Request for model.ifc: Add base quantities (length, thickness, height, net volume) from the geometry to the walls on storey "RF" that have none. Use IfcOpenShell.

First a look at what the model holds.

```python
import ifcopenshell
import ifcopenshell.util.element
import ifcopenshell.util.unit

model = ifcopenshell.open("model.ifc")
print(model.schema)
for unit_type in ("LENGTHUNIT", "AREAUNIT", "VOLUMEUNIT"):
    print(unit_type, ifcopenshell.util.unit.calculate_unit_scale(model, unit_type))
storey = next(s for s in model.by_type("IfcBuildingStorey") if s.Name == "RF")
walls = [e for e in ifcopenshell.util.element.get_decomposition(storey) if e.is_a("IfcWall")]
for e in sorted(walls, key=lambda e: e.id()):
    print(e.id(), e.is_a(), e.Name, list(ifcopenshell.util.element.get_psets(e, qtos_only=True)), sep=" | ")
```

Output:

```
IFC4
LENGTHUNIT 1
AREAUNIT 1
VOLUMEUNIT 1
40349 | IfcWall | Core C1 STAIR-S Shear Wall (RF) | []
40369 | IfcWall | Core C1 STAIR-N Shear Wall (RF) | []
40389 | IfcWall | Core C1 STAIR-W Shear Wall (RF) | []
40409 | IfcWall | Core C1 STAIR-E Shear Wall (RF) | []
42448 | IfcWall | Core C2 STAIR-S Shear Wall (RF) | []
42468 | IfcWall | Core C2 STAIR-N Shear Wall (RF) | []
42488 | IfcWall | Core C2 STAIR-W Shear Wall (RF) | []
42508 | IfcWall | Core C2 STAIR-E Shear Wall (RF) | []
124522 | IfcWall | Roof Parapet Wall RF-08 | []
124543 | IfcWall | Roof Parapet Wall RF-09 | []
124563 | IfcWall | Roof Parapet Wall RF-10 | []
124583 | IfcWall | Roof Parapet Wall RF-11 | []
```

```python
import ifcopenshell
import ifcopenshell.api.pset
import ifcopenshell.geom
import ifcopenshell.util.element
import ifcopenshell.util.shape
import ifcopenshell.util.unit

model = ifcopenshell.open("model.ifc")
unit_scale = ifcopenshell.util.unit.calculate_unit_scale(model)
volume_scale = ifcopenshell.util.unit.calculate_unit_scale(model, "VOLUMEUNIT")
settings = ifcopenshell.geom.settings()

storey = next(s for s in model.by_type("IfcBuildingStorey") if s.Name == "RF")
walls = [e for e in ifcopenshell.util.element.get_decomposition(storey) if e.is_a("IfcWall")]

for e in sorted(walls, key=lambda e: e.id()):
    if ifcopenshell.util.element.get_psets(e, qtos_only=True, should_inherit=False):
        continue
    # Geometry comes back in metres, in the element's own axes.
    shape = ifcopenshell.geom.create_shape(settings, e)
    values = {
        "Length": ifcopenshell.util.shape.get_x(shape.geometry) / unit_scale,
        "Width": ifcopenshell.util.shape.get_y(shape.geometry) / unit_scale,
        "Height": ifcopenshell.util.shape.get_z(shape.geometry) / unit_scale,
        "NetVolume": ifcopenshell.util.shape.get_volume(shape.geometry) / volume_scale,
    }
    qto = ifcopenshell.api.pset.add_qto(model, product=e, name="Qto_WallBaseQuantities")
    ifcopenshell.api.pset.edit_qto(model, qto=qto, properties=values)
    print(e.id(), {k: round(v, 3) for k, v in values.items()})

model.write("model-out.ifc")
```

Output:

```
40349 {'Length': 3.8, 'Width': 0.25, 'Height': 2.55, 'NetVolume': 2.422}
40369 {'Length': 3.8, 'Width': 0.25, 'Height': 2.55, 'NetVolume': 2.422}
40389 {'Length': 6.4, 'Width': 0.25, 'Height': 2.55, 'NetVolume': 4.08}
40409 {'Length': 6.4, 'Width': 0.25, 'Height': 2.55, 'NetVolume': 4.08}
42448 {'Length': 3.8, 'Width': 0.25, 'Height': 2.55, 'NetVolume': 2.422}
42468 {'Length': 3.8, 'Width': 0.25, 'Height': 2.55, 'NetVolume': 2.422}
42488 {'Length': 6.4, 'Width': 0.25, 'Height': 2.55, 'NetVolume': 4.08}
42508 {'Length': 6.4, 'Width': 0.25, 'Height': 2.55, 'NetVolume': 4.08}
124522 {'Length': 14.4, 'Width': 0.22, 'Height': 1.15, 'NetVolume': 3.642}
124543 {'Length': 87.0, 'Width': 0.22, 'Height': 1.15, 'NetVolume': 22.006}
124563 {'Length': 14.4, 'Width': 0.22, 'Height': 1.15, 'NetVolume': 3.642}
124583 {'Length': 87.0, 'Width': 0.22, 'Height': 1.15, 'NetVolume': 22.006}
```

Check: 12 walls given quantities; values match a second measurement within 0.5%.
